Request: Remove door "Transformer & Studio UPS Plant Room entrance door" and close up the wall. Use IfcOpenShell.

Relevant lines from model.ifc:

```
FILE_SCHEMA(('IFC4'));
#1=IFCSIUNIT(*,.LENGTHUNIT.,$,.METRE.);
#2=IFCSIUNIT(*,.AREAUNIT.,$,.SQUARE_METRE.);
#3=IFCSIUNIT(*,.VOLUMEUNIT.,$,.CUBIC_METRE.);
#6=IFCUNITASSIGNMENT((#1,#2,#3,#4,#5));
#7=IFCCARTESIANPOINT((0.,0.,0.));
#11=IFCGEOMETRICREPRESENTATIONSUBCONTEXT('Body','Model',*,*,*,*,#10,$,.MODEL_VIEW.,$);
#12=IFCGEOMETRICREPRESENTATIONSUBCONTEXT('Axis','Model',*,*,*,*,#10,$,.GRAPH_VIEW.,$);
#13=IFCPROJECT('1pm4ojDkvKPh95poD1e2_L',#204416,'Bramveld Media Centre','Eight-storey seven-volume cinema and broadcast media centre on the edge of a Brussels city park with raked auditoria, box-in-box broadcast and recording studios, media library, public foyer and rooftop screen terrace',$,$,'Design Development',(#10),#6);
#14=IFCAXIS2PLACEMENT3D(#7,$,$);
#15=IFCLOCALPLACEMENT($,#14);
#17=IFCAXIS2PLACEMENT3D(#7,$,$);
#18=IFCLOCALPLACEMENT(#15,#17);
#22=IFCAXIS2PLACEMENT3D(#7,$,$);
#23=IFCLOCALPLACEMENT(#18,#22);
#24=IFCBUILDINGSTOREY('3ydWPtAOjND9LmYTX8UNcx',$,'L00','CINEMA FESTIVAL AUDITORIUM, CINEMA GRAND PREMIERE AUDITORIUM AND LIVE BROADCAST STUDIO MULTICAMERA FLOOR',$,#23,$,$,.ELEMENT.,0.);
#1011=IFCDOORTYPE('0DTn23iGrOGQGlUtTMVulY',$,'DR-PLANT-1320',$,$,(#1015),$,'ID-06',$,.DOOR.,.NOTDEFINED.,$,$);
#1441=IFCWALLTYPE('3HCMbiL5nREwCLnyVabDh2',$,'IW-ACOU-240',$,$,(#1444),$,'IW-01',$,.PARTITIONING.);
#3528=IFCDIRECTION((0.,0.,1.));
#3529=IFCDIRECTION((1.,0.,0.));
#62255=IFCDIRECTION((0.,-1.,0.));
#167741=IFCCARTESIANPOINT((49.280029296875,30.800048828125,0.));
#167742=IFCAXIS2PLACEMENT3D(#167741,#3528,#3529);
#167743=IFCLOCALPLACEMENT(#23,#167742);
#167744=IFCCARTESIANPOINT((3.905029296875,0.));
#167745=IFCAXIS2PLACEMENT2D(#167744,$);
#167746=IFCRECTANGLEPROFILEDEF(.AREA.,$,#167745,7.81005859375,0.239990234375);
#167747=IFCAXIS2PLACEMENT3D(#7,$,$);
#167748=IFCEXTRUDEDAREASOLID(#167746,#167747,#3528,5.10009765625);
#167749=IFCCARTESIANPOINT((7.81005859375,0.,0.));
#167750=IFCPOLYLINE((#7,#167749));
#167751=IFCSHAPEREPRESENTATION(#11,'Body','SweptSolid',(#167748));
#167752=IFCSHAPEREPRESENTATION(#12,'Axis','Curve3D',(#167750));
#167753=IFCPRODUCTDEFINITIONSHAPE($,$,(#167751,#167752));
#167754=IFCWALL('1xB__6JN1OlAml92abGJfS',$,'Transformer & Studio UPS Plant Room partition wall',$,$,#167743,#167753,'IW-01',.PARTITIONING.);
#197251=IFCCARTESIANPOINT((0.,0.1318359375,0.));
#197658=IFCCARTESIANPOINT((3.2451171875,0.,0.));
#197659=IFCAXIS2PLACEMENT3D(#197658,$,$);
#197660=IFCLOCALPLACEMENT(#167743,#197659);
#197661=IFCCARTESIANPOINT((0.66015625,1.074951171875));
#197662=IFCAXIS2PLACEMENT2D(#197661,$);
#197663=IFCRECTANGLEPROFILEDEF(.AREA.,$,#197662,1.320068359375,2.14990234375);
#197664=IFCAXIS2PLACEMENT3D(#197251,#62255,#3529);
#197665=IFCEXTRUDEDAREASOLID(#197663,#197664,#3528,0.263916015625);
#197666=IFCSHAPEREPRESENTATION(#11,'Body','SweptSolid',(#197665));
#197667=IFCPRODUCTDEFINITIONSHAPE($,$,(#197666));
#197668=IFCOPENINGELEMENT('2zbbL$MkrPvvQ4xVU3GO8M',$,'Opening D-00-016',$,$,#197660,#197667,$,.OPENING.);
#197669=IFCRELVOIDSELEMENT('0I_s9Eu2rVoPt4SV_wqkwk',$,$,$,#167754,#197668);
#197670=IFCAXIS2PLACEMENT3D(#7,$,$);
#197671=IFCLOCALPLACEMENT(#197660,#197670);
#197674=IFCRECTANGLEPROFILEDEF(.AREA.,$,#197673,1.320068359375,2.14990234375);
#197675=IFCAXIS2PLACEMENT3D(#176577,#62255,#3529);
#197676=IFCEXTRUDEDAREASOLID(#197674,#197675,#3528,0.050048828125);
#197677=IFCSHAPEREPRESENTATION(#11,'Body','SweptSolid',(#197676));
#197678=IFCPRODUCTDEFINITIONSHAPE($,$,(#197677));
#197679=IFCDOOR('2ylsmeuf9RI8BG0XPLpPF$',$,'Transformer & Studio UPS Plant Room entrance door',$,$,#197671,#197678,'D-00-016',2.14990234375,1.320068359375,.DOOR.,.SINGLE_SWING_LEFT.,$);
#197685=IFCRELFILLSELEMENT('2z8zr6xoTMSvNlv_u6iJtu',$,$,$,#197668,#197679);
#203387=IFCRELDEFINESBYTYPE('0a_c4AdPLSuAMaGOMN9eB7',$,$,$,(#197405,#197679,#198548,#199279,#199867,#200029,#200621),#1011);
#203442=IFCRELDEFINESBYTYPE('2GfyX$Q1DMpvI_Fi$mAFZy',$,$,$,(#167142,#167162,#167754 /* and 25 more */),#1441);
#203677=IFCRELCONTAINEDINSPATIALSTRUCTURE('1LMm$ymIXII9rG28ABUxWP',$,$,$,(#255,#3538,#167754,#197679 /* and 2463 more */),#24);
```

```python
import ifcopenshell
import ifcopenshell.api.feature
import ifcopenshell.api.root
import ifcopenshell.geom
import ifcopenshell.util.shape

model = ifcopenshell.open("model.ifc")
settings = ifcopenshell.geom.settings()


def volume(element):
    """Net volume in cubic metres, openings subtracted."""
    shape = ifcopenshell.geom.create_shape(settings, element)
    return ifcopenshell.util.shape.get_volume(shape.geometry)


door = model.by_guid("2ylsmeuf9RI8BG0XPLpPF$")
opening = door.FillsVoids[0].RelatingOpeningElement
wall = opening.VoidsElements[0].RelatingBuildingElement
before = volume(wall)

ifcopenshell.api.root.remove_product(model, product=door)
ifcopenshell.api.feature.remove_feature(model, feature=opening)

after = volume(wall)

print(f"wall volume {before:.3f} -> {after:.3f} m3")

model.write("model-out.ifc")
```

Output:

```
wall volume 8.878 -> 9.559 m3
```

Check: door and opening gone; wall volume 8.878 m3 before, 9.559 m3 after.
